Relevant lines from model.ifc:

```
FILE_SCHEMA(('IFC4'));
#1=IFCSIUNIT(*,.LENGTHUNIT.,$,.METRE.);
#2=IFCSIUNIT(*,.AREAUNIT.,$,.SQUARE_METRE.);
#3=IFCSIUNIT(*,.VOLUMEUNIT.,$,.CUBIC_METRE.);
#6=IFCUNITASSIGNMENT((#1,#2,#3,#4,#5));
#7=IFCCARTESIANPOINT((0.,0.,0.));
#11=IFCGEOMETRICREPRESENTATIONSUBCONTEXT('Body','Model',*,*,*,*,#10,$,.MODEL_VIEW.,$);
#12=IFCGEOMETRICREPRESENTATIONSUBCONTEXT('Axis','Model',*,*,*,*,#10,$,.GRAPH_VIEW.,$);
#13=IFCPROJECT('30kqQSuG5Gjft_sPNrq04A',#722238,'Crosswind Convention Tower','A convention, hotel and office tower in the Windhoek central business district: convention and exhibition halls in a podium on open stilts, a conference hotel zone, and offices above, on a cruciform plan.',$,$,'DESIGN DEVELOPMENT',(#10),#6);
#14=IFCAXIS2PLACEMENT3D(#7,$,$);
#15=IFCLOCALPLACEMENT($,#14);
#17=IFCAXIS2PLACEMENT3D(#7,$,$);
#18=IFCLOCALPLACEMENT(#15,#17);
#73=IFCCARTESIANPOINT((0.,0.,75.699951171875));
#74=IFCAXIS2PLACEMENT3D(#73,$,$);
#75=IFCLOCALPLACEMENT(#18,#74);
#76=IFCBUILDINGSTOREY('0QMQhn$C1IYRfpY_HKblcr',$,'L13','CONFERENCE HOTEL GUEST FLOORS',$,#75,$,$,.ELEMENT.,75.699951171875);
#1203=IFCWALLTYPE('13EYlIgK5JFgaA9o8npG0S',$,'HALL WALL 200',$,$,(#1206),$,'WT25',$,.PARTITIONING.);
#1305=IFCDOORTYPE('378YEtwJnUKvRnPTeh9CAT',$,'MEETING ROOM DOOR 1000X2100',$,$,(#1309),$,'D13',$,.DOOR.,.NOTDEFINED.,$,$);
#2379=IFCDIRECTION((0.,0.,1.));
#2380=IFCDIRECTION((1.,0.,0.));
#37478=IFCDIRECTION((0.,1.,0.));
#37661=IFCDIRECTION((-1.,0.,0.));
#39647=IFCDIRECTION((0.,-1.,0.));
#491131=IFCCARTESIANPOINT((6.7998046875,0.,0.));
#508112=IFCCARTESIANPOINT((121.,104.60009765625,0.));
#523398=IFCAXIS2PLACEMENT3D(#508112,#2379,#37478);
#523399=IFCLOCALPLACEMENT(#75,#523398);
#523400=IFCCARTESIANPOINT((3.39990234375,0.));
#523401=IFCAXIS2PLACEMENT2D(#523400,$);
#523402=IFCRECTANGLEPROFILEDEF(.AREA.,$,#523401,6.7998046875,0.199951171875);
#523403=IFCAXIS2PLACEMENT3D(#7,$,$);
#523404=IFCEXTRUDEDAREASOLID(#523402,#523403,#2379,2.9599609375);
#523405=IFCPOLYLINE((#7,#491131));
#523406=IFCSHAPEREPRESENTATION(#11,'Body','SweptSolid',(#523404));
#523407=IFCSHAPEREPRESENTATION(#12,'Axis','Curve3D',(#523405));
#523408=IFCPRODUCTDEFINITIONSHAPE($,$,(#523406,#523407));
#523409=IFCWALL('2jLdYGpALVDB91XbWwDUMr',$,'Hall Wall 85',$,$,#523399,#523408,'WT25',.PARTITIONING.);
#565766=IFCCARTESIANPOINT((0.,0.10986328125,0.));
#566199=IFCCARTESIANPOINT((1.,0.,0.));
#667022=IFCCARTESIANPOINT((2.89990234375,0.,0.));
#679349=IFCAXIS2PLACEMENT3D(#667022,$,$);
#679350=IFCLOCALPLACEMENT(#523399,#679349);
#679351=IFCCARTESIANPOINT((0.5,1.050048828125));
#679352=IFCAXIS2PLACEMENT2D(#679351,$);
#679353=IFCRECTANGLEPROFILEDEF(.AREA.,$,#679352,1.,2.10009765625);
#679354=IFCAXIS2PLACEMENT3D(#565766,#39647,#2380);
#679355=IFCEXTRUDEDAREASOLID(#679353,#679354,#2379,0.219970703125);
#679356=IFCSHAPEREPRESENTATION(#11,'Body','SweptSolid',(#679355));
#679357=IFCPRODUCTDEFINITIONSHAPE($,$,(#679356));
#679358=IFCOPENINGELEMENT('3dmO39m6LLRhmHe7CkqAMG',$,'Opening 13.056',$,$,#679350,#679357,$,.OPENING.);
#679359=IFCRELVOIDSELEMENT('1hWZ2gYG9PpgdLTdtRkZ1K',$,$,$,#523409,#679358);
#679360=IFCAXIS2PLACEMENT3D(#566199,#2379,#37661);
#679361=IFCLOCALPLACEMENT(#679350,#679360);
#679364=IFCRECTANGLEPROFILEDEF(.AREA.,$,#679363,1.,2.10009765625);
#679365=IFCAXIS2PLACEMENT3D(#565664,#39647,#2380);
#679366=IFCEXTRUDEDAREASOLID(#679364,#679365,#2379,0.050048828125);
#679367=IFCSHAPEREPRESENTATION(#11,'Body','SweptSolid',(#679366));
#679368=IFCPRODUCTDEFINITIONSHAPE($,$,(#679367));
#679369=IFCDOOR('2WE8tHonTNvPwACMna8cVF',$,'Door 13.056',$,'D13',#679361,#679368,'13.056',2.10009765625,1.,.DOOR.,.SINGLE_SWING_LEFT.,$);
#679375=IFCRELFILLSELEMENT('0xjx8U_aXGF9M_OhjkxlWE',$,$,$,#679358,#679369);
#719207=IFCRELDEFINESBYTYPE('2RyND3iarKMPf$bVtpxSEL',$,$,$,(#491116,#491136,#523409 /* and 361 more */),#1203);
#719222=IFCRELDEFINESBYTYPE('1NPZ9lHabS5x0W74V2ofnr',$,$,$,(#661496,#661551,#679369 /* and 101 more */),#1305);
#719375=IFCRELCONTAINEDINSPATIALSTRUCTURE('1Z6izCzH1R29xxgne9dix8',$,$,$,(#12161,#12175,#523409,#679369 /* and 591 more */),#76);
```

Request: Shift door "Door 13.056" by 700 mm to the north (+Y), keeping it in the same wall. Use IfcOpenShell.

```python
import ifcopenshell
import ifcopenshell.api.geometry
import ifcopenshell.util.placement
import ifcopenshell.util.unit

model = ifcopenshell.open("model.ifc")
unit_scale = ifcopenshell.util.unit.calculate_unit_scale(model)

door = model.by_guid("2WE8tHonTNvPwACMna8cVF")
opening = door.FillsVoids[0].RelatingOpeningElement
wall = opening.VoidsElements[0].RelatingBuildingElement

wall_matrix = ifcopenshell.util.placement.get_local_placement(wall.ObjectPlacement)
shift = wall_matrix[:3, 0] * 0.7 / unit_scale
before = ifcopenshell.util.placement.get_local_placement(door.ObjectPlacement)[:3, 3].copy()

# The door is placed relative to its opening, so it follows when the opening moves.
matrix = ifcopenshell.util.placement.get_local_placement(opening.ObjectPlacement)
matrix[:3, 3] += shift
ifcopenshell.api.geometry.edit_object_placement(
    model, product=opening, matrix=matrix, is_si=False, should_transform_children=True
)

after = ifcopenshell.util.placement.get_local_placement(door.ObjectPlacement)[:3, 3]
print("door moved by", (after - before).round(3) + 0.0)

model.write("model_rev.ifc")
```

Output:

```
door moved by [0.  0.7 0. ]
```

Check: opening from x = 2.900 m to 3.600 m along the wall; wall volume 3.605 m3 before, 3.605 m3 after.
